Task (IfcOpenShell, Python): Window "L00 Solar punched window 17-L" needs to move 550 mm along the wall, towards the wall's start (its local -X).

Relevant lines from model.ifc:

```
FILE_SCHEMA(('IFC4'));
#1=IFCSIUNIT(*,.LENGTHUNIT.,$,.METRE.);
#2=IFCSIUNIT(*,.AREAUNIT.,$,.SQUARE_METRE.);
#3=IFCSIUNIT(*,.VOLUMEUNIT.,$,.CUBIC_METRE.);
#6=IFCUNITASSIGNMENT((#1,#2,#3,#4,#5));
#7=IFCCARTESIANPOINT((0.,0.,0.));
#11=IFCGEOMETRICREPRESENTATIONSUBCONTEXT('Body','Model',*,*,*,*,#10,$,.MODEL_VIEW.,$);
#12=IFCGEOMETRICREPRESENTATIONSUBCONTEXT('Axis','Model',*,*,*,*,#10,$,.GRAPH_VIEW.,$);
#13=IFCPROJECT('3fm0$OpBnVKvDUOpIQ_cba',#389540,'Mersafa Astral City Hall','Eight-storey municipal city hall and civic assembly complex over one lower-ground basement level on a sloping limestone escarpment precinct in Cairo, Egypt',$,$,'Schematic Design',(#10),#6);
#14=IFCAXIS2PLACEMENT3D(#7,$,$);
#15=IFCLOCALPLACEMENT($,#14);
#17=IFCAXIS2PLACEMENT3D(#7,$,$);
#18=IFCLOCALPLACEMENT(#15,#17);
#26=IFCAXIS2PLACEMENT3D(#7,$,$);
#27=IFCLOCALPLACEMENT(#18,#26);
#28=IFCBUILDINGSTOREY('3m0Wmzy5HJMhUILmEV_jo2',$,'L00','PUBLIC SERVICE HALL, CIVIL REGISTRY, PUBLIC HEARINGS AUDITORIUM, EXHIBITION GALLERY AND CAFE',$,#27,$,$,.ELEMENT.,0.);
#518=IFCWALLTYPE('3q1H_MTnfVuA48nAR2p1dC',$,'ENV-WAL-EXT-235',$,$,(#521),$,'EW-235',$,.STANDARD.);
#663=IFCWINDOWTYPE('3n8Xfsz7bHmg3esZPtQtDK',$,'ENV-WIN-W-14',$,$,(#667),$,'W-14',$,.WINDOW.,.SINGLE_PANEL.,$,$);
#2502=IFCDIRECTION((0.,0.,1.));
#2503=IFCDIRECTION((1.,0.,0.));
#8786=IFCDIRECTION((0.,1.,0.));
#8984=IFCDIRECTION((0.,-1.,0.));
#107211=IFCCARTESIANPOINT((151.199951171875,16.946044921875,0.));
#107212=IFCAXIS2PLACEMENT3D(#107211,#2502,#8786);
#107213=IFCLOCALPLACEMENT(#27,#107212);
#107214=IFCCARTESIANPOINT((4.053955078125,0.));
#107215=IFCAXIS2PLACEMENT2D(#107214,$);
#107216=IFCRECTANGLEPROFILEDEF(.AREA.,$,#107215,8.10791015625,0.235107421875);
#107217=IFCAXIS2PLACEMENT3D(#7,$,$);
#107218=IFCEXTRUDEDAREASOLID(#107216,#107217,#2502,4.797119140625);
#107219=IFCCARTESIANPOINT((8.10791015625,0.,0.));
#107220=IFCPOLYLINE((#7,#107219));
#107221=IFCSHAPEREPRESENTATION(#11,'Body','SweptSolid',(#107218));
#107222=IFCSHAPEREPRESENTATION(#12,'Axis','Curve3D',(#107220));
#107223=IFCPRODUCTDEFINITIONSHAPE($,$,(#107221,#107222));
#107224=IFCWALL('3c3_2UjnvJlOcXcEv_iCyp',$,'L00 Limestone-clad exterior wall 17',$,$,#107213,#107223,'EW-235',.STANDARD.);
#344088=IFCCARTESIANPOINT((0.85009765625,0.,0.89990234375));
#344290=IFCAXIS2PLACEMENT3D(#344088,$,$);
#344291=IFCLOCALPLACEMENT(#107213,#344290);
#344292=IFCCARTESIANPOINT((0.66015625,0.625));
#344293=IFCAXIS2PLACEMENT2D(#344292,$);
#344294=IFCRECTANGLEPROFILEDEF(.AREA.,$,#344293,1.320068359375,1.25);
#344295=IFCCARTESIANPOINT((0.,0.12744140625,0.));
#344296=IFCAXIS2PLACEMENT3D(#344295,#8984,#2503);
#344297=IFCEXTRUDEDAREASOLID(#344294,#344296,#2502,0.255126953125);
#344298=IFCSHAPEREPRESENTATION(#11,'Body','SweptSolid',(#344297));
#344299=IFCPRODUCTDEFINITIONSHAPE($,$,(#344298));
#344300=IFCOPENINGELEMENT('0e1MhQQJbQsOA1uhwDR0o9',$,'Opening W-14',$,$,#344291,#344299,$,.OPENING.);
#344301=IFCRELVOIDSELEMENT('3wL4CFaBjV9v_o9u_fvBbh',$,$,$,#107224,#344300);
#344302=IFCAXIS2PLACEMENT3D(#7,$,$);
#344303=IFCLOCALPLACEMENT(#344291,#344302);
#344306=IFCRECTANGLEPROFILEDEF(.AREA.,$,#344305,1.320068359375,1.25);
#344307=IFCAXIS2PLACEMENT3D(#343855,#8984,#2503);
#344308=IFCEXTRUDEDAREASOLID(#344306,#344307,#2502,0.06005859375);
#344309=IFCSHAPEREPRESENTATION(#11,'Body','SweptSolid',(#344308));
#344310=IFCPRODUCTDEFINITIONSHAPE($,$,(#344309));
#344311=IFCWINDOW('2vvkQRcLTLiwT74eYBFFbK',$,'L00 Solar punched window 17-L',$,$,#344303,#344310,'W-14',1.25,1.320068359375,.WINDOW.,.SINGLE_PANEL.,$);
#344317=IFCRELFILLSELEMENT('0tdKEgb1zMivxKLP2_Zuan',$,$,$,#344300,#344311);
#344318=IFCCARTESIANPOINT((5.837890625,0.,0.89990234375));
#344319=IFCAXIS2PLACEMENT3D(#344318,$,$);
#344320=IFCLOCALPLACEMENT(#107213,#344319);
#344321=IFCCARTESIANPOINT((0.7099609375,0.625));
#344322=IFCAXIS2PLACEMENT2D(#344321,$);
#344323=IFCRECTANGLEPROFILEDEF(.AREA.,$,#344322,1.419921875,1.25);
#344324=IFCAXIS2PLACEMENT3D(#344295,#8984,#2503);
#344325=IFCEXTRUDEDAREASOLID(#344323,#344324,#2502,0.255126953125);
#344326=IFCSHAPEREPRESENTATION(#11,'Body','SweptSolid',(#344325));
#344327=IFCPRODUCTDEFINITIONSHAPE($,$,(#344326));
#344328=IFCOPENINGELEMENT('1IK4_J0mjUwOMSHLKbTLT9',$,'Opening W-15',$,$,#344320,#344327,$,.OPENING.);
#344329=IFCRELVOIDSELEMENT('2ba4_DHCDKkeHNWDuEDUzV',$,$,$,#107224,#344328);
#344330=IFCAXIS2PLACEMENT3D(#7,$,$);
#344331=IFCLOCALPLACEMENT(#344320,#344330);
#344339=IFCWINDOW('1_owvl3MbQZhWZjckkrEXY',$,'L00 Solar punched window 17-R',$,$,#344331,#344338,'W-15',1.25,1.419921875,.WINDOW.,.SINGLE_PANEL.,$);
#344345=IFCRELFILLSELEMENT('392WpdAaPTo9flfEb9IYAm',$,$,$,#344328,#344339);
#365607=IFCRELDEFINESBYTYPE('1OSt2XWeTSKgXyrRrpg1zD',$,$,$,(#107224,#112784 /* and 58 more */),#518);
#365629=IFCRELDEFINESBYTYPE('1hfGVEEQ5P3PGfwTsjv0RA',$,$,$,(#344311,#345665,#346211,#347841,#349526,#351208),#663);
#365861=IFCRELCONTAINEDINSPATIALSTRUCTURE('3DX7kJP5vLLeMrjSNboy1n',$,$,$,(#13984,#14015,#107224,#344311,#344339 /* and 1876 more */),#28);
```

```python
import ifcopenshell
import ifcopenshell.api.geometry
import ifcopenshell.util.placement
import ifcopenshell.util.unit

model = ifcopenshell.open("model.ifc")
unit_scale = ifcopenshell.util.unit.calculate_unit_scale(model)

window = model.by_guid("2vvkQRcLTLiwT74eYBFFbK")
opening = window.FillsVoids[0].RelatingOpeningElement
wall = opening.VoidsElements[0].RelatingBuildingElement

wall_matrix = ifcopenshell.util.placement.get_local_placement(wall.ObjectPlacement)
shift = wall_matrix[:3, 0] * -0.55 / unit_scale
before = ifcopenshell.util.placement.get_local_placement(window.ObjectPlacement)[:3, 3].copy()

# The window is placed relative to its opening, so it follows when the opening moves.
matrix = ifcopenshell.util.placement.get_local_placement(opening.ObjectPlacement)
matrix[:3, 3] += shift
ifcopenshell.api.geometry.edit_object_placement(
    model, product=opening, matrix=matrix, is_si=False, should_transform_children=True
)

after = ifcopenshell.util.placement.get_local_placement(window.ObjectPlacement)[:3, 3]
print("window moved by", (after - before).round(3) + 0.0)

model.write("model_v2.ifc")
```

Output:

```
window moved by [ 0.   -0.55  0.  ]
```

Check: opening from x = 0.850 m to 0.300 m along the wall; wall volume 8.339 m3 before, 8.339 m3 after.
